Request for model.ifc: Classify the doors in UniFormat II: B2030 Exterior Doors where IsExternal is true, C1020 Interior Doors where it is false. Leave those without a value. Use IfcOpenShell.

First a look at what the model holds.

```python
import ifcopenshell
import ifcopenshell.util.element

model = ifcopenshell.open("model.ifc")
print(model.schema)
print("classifications:", [c.Name for c in model.by_type("IfcClassification")])
values = [ifcopenshell.util.element.get_pset(e, "Pset_DoorCommon", "IsExternal") for e in model.by_type("IfcDoor")]
for value in (True, False, None):
    print("IsExternal", value, values.count(value))
```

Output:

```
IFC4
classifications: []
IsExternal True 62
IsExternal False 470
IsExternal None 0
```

```python
import ifcopenshell
import ifcopenshell.api.classification
import ifcopenshell.util.element

model = ifcopenshell.open("model.ifc")

system = ifcopenshell.api.classification.add_classification(model, classification="UniFormat II")

doors = model.by_type("IfcDoor")
external = {e: ifcopenshell.util.element.get_pset(e, "Pset_DoorCommon", "IsExternal") for e in doors}
for flag, code, name in ((True, "B2030", "Exterior Doors"), (False, "C1020", "Interior Doors")):
    products = [e for e in doors if external[e] is flag]
    ifcopenshell.api.classification.add_reference(
        model, products=products, classification=system, identification=code, name=name
    )
    print(code, len(products))

model.write("model_updated.ifc")
```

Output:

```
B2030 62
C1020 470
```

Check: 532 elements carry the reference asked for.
